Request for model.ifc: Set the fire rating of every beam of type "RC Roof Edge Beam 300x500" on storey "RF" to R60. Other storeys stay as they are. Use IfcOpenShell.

First a look at what the model holds.

```python
import ifcopenshell
import ifcopenshell.util.element

model = ifcopenshell.open("model.ifc")
print(model.schema)
storey = next(s for s in model.by_type("IfcBuildingStorey") if s.Name == "RF")
beams = [e for e in ifcopenshell.util.element.get_decomposition(storey) if e.is_a("IfcBeam")]
seen = {}
for e in beams:
    element_type = ifcopenshell.util.element.get_type(e)
    key = (element_type.Name if element_type != e and element_type else None, ifcopenshell.util.element.get_pset(e, "Pset_BeamCommon", "FireRating"))
    seen[key] = seen.get(key, 0) + 1
for (name, value), count in sorted(seen.items(), key=str):
    print(count, "x", name, "|", value)
```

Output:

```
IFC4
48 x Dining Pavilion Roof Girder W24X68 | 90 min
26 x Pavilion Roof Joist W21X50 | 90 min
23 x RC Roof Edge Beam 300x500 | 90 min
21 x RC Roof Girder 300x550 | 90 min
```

```python
import ifcopenshell
import ifcopenshell.api.pset
import ifcopenshell.util.element

model = ifcopenshell.open("model.ifc")

storey = next(s for s in model.by_type("IfcBuildingStorey") if s.Name == "RF")
beams = [e for e in ifcopenshell.util.element.get_decomposition(storey) if e.is_a("IfcBeam")]

count = 0
for e in beams:
    element_type = ifcopenshell.util.element.get_type(e)
    if element_type in (None, e) or element_type.Name != "RC Roof Edge Beam 300x500":
        continue
    # add_pset returns the element's existing set when there is one.
    pset = ifcopenshell.api.pset.add_pset(model, product=e, name="Pset_BeamCommon")
    ifcopenshell.api.pset.edit_pset(model, pset=pset, properties={"FireRating": "R60"})
    count += 1

print(count, "beams updated")

model.write("model_updated.ifc")
```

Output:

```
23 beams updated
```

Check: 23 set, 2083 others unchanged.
